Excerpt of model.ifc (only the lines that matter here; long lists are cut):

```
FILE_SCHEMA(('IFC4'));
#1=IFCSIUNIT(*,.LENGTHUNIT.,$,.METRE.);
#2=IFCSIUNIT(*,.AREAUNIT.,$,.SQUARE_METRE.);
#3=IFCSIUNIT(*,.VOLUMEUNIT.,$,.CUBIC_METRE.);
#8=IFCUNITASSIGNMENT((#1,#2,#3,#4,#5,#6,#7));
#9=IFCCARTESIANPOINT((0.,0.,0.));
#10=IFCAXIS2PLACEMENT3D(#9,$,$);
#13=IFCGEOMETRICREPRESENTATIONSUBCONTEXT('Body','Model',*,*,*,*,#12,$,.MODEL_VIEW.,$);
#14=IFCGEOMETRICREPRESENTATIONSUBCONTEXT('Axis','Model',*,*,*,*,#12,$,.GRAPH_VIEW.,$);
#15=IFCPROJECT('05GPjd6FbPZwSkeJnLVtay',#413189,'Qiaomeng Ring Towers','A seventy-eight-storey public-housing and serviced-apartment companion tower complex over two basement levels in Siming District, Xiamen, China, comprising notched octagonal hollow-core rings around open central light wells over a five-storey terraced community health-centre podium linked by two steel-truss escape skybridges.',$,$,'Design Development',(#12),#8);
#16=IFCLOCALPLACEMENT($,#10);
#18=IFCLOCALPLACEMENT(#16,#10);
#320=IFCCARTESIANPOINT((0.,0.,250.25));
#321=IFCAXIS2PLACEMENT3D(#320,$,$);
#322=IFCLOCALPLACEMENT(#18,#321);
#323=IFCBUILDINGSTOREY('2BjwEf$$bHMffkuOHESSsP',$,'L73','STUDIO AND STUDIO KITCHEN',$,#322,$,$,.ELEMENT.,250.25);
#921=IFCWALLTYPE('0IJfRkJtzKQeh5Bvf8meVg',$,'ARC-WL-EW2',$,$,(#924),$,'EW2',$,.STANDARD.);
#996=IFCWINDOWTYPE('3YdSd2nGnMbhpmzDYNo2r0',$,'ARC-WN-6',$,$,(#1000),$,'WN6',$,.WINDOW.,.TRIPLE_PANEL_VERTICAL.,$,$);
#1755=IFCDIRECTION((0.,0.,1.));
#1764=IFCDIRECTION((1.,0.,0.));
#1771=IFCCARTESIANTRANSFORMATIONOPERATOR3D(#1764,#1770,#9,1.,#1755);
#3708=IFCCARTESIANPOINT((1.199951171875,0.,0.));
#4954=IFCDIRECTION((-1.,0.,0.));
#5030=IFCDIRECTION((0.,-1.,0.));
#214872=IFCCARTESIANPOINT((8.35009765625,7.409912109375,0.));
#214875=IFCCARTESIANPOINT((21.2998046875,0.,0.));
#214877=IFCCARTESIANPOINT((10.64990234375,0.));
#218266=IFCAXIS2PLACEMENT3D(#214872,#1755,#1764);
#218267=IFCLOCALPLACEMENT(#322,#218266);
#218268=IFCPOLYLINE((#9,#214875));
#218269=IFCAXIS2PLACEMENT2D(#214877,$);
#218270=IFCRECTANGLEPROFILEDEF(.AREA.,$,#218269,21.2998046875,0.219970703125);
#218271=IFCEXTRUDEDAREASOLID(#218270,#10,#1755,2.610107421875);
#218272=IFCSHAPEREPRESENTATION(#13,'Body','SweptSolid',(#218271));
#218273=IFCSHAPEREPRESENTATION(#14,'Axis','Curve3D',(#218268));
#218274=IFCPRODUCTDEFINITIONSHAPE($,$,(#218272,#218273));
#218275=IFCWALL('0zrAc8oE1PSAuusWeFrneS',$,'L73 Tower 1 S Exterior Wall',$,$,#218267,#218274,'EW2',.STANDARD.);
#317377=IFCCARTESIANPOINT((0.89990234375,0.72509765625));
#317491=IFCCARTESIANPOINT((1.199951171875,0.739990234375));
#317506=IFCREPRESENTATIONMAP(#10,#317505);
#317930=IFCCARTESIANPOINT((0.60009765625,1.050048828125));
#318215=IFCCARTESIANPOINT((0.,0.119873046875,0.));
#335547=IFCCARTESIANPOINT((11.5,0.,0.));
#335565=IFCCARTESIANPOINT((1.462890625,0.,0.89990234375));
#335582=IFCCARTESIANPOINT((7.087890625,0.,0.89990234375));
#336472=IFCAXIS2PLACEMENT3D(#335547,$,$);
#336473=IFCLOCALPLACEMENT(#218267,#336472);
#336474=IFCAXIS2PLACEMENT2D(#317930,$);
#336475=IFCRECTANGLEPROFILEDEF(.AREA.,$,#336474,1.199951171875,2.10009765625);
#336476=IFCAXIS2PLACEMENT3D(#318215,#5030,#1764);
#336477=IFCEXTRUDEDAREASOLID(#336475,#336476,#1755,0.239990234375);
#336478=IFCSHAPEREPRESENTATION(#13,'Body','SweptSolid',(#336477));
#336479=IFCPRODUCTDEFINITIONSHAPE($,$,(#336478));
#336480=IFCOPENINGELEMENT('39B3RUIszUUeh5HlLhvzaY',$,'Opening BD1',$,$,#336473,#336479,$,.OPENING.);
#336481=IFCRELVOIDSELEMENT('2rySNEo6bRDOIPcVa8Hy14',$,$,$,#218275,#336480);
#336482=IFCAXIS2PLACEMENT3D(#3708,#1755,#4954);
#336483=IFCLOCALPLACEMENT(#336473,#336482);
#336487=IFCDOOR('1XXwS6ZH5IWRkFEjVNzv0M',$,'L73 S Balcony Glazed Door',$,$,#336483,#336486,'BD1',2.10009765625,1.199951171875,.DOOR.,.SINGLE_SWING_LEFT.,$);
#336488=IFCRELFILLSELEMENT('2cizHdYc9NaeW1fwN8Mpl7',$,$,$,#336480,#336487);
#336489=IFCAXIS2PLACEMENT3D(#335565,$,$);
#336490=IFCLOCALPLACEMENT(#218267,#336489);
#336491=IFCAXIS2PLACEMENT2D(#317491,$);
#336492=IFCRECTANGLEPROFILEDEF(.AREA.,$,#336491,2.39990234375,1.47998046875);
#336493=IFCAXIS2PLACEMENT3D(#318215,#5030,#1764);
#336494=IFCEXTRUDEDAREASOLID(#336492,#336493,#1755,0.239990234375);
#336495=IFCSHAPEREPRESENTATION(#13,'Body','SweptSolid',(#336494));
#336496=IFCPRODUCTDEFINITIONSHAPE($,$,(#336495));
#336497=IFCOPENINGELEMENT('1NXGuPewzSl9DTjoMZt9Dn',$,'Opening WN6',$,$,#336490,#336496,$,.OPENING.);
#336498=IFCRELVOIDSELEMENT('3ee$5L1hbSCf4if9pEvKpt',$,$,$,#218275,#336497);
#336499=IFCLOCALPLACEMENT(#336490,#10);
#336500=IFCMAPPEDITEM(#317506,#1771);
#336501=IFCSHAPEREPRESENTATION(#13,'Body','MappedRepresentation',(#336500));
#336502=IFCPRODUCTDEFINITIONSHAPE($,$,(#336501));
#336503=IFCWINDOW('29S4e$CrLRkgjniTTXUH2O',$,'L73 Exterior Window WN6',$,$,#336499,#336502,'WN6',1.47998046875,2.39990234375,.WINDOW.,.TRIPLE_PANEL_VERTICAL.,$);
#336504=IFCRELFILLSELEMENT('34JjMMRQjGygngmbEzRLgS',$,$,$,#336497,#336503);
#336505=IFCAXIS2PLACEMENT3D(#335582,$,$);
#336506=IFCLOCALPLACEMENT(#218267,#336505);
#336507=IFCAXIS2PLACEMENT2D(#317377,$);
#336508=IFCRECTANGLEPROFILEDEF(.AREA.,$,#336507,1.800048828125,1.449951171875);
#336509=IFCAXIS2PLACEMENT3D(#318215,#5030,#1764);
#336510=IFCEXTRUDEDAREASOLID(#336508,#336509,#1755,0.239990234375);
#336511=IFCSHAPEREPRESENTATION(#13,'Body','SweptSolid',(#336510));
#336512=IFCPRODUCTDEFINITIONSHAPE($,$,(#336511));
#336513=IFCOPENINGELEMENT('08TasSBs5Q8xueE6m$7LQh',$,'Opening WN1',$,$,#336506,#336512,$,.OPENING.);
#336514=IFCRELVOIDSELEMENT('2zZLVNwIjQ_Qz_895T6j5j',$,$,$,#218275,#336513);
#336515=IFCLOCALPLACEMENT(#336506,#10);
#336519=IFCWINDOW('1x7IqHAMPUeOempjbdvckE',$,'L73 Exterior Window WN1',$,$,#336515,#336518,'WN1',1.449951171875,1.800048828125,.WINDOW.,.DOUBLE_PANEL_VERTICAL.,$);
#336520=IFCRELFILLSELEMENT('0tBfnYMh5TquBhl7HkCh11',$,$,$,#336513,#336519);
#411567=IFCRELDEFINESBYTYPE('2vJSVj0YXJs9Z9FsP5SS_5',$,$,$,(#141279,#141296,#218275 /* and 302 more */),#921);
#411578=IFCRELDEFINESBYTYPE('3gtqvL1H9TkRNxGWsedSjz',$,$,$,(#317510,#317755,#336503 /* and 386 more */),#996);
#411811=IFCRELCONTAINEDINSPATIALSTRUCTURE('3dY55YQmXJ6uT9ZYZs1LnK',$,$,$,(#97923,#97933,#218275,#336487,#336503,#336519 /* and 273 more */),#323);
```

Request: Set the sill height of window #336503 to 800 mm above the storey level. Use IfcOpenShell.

```python
import numpy as np
import ifcopenshell
import ifcopenshell.api.geometry
import ifcopenshell.geom
import ifcopenshell.util.element
import ifcopenshell.util.placement
import ifcopenshell.util.shape
import ifcopenshell.util.unit

model = ifcopenshell.open("model.ifc")
unit_scale = ifcopenshell.util.unit.calculate_unit_scale(model)

window = model.by_guid("29S4e$CrLRkgjniTTXUH2O")
opening = window.FillsVoids[0].RelatingOpeningElement
storey = ifcopenshell.util.element.get_container(window, ifc_class="IfcBuildingStorey")
level = ifcopenshell.util.placement.get_local_placement(storey.ObjectPlacement)[2, 3]

# The opening's origin need not be at the sill, so measure its lowest point.
shape = ifcopenshell.geom.create_shape(ifcopenshell.geom.settings(), opening)
bottom = ifcopenshell.util.shape.get_shape_bottom_elevation(shape, shape.geometry) / unit_scale
dz = level + 0.8 - bottom

shift = np.array([0.0, 0.0, dz])
# The window is placed relative to its opening, so it follows when the opening moves.
matrix = ifcopenshell.util.placement.get_local_placement(opening.ObjectPlacement)
matrix[:3, 3] += shift
ifcopenshell.api.geometry.edit_object_placement(
    model, product=opening, matrix=matrix, is_si=False, should_transform_children=True
)

print(f"moved by {dz * unit_scale:+.3f} m")

model.write("model_v2.ifc")
```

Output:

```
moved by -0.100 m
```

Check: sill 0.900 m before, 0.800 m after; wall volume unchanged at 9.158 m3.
